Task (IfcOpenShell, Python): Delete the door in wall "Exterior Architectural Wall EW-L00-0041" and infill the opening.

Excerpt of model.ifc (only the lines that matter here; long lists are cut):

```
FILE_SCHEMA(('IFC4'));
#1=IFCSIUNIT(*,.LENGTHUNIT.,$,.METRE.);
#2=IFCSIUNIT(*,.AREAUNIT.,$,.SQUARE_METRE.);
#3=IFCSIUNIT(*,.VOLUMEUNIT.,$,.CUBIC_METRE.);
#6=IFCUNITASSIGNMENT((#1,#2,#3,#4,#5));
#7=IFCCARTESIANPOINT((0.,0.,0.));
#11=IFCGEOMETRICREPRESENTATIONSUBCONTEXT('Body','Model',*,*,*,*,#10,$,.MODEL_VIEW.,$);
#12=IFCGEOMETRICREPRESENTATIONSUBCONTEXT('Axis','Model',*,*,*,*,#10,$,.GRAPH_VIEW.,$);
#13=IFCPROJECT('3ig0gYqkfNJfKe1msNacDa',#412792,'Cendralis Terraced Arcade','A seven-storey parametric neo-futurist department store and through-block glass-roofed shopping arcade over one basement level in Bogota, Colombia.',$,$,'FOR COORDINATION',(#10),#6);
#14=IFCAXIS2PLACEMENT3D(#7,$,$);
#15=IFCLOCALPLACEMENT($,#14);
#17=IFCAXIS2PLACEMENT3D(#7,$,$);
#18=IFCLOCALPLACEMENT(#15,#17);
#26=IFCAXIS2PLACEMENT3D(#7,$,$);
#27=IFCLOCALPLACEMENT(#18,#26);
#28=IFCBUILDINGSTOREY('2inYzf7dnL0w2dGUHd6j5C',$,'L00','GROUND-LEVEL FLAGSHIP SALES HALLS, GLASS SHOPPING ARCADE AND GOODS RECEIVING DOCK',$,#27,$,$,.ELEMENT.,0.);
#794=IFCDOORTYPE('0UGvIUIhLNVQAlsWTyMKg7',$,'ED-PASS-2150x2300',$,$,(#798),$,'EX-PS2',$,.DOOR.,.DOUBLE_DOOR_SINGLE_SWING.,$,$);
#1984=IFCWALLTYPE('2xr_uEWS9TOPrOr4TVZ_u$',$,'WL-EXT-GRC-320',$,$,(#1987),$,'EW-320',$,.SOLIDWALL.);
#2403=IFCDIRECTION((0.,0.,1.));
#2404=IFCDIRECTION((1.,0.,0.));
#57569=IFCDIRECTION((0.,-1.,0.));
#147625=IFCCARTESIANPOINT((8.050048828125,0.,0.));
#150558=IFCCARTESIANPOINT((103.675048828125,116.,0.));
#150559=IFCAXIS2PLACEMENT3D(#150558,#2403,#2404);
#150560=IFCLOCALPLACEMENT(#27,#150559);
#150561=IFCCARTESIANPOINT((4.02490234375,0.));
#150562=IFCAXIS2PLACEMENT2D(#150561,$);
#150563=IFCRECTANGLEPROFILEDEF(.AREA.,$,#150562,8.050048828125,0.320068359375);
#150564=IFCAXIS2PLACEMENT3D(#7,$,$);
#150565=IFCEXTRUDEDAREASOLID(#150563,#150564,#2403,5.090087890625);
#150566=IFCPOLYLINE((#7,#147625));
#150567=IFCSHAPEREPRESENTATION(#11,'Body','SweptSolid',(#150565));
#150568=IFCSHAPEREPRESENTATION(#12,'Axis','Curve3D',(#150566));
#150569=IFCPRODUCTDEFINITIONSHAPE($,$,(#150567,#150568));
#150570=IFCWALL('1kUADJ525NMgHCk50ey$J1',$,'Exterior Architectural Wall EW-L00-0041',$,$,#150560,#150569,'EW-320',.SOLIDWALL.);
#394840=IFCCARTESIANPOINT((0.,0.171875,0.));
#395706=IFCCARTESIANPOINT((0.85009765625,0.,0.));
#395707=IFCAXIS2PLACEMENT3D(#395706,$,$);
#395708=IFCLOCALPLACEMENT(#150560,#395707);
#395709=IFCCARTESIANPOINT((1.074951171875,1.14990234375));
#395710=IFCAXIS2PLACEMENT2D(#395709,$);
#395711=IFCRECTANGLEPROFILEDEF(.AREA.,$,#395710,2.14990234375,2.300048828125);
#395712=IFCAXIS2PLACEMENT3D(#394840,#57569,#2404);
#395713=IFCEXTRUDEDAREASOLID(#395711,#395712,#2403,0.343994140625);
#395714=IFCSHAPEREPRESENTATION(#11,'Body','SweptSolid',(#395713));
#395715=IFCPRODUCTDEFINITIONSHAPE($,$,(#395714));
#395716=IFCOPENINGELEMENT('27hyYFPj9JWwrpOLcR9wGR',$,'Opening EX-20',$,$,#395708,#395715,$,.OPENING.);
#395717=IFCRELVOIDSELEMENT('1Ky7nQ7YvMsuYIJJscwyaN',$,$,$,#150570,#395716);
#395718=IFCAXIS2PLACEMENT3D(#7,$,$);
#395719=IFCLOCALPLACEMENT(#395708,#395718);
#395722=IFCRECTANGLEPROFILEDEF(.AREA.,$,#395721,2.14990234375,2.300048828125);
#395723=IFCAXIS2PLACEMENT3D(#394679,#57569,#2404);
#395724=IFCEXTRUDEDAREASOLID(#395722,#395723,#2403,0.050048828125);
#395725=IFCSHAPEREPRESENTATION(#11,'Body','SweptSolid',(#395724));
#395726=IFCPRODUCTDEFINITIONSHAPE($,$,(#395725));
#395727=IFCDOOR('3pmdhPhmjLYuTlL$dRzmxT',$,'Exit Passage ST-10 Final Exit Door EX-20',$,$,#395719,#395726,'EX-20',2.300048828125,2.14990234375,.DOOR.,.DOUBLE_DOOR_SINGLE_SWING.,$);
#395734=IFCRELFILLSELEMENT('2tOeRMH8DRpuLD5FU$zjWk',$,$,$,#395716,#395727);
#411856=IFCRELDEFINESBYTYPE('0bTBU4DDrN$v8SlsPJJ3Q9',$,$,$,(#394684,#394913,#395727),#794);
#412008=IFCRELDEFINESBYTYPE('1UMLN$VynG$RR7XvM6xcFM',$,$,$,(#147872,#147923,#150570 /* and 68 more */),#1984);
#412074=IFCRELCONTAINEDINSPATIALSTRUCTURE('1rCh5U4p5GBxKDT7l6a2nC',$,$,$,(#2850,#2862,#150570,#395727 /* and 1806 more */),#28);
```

```python
import ifcopenshell
import ifcopenshell.api.feature
import ifcopenshell.api.root
import ifcopenshell.geom
import ifcopenshell.util.shape

model = ifcopenshell.open("model.ifc")
settings = ifcopenshell.geom.settings()


def volume(element):
    """Net volume in cubic metres, openings subtracted."""
    shape = ifcopenshell.geom.create_shape(settings, element)
    return ifcopenshell.util.shape.get_volume(shape.geometry)


door = model.by_guid("3pmdhPhmjLYuTlL$dRzmxT")
opening = door.FillsVoids[0].RelatingOpeningElement
wall = opening.VoidsElements[0].RelatingBuildingElement
before = volume(wall)

ifcopenshell.api.root.remove_product(model, product=door)
ifcopenshell.api.feature.remove_feature(model, feature=opening)

after = volume(wall)

print(f"wall volume {before:.3f} -> {after:.3f} m3")

model.write("model_updated.ifc")
```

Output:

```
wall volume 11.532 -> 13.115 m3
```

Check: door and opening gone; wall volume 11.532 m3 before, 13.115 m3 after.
